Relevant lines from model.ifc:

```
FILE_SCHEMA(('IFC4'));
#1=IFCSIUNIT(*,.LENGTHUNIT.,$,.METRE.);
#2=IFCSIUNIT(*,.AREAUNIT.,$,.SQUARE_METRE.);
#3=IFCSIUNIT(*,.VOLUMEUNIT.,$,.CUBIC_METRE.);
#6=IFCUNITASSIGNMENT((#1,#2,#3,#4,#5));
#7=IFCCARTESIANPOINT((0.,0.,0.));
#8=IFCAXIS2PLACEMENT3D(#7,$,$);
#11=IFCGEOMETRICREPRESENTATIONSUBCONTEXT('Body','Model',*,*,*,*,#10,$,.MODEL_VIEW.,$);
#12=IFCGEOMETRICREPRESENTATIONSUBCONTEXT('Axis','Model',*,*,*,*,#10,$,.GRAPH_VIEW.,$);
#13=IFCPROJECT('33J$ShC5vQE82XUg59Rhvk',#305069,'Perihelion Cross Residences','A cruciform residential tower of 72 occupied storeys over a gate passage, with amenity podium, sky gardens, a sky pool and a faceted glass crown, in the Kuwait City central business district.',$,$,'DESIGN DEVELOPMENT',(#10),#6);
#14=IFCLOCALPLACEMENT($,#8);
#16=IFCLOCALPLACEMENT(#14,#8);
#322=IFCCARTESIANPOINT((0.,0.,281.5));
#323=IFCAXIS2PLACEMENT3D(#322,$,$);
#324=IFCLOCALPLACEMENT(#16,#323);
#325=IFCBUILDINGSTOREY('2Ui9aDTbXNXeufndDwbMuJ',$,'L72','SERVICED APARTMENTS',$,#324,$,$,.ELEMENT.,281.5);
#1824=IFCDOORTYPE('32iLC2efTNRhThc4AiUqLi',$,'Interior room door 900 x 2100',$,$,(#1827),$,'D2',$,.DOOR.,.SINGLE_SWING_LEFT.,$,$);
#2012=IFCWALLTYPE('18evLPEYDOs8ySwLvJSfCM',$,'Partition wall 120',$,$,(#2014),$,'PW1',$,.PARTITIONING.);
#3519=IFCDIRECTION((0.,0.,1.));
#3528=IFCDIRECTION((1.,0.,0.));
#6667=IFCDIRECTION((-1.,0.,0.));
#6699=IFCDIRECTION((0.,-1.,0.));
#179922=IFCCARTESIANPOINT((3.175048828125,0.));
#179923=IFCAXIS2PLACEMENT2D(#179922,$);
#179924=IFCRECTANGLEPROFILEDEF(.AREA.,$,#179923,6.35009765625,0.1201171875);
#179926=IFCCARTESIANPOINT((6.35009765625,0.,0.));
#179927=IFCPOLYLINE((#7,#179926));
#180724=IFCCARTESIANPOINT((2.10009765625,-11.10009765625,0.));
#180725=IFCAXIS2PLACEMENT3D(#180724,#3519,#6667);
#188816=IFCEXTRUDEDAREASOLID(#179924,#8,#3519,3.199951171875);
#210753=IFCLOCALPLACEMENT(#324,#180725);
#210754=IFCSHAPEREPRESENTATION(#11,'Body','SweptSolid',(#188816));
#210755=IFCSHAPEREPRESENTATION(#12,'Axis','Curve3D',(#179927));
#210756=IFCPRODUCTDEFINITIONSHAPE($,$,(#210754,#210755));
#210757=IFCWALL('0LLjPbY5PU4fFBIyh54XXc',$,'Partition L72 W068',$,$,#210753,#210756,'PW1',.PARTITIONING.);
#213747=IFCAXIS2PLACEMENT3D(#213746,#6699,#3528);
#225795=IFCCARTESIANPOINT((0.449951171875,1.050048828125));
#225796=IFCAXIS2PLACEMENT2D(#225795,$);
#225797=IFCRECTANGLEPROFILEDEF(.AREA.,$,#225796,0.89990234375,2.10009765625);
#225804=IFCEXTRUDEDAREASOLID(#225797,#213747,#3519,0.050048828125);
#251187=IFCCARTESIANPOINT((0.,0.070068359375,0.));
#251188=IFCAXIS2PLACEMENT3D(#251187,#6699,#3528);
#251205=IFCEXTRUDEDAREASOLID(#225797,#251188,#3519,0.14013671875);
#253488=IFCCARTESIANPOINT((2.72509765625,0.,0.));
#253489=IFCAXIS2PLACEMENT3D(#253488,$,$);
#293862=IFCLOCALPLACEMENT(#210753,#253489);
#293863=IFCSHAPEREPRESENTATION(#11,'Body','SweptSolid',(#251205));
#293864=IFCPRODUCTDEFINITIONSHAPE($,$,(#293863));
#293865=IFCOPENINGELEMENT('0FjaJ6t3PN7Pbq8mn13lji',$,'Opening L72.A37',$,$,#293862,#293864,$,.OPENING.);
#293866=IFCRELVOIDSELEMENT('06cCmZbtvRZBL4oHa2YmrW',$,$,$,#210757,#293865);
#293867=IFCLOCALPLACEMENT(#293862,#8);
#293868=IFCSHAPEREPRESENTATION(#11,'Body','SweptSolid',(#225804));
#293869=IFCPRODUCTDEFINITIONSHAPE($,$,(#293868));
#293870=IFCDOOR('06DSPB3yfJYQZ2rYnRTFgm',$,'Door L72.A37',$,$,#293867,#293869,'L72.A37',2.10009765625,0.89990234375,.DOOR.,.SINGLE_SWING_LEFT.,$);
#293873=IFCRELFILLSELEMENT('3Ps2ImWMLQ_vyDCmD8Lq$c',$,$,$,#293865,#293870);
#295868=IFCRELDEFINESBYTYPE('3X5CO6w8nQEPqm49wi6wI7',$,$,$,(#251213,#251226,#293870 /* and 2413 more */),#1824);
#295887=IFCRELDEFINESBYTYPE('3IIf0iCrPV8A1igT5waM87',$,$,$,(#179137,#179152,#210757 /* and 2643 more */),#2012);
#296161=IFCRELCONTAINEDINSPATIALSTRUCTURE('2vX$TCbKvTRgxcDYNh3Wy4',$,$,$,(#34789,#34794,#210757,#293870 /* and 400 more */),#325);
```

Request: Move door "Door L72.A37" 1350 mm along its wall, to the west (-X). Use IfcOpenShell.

```python
import ifcopenshell
import ifcopenshell.api.geometry
import ifcopenshell.util.placement

model = ifcopenshell.open("model.ifc")

door = model.by_guid("06DSPB3yfJYQZ2rYnRTFgm")
opening = door.FillsVoids[0].RelatingOpeningElement
wall = opening.VoidsElements[0].RelatingBuildingElement

wall_matrix = ifcopenshell.util.placement.get_local_placement(wall.ObjectPlacement)
shift = wall_matrix[:3, 0] * 1.35
before = ifcopenshell.util.placement.get_local_placement(door.ObjectPlacement)[:3, 3].copy()

# The door is placed relative to its opening, so it follows when the opening moves.
matrix = ifcopenshell.util.placement.get_local_placement(opening.ObjectPlacement)
matrix[:3, 3] += shift
ifcopenshell.api.geometry.edit_object_placement(
    model, product=opening, matrix=matrix, is_si=False, should_transform_children=True
)

after = ifcopenshell.util.placement.get_local_placement(door.ObjectPlacement)[:3, 3]
print("door moved by", (after - before).round(3) + 0.0)

model.write("model_v2.ifc")
```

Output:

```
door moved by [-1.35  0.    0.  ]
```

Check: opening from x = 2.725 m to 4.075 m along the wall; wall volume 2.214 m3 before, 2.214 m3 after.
